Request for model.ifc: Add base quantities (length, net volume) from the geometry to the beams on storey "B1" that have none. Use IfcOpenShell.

First a look at what the model holds.

```python
import ifcopenshell
import ifcopenshell.util.element
import ifcopenshell.util.unit

model = ifcopenshell.open("model.ifc")
print(model.schema)
for unit_type in ("LENGTHUNIT", "AREAUNIT", "VOLUMEUNIT"):
    print(unit_type, ifcopenshell.util.unit.calculate_unit_scale(model, unit_type))
storey = next(s for s in model.by_type("IfcBuildingStorey") if s.Name == "B1")
beams = [e for e in ifcopenshell.util.element.get_decomposition(storey) if e.is_a("IfcBeam")]
for e in sorted(beams, key=lambda e: e.id()):
    print(e.id(), e.is_a(), e.Name, list(ifcopenshell.util.element.get_psets(e, qtos_only=True)), sep=" | ")
```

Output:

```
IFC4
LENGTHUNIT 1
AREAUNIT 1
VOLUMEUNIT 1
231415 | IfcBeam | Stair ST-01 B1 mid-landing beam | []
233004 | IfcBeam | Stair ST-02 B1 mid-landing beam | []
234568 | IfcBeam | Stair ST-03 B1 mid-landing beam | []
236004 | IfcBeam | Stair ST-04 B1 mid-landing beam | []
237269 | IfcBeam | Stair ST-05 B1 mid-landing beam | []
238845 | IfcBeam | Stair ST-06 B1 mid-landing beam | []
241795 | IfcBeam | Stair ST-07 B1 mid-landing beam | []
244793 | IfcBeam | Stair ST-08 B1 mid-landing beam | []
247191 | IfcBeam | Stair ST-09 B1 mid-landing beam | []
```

```python
import ifcopenshell
import ifcopenshell.api.pset
import ifcopenshell.geom
import ifcopenshell.util.element
import ifcopenshell.util.shape
import ifcopenshell.util.unit

model = ifcopenshell.open("model.ifc")
unit_scale = ifcopenshell.util.unit.calculate_unit_scale(model)
volume_scale = ifcopenshell.util.unit.calculate_unit_scale(model, "VOLUMEUNIT")
settings = ifcopenshell.geom.settings()

storey = next(s for s in model.by_type("IfcBuildingStorey") if s.Name == "B1")
beams = [e for e in ifcopenshell.util.element.get_decomposition(storey) if e.is_a("IfcBeam")]

for e in sorted(beams, key=lambda e: e.id()):
    if ifcopenshell.util.element.get_psets(e, qtos_only=True, should_inherit=False):
        continue
    # Geometry comes back in metres, in the element's own axes.
    shape = ifcopenshell.geom.create_shape(settings, e)
    values = {
        "Length": ifcopenshell.util.shape.get_max_xyz(shape.geometry) / unit_scale,
        "NetVolume": ifcopenshell.util.shape.get_volume(shape.geometry) / volume_scale,
    }
    qto = ifcopenshell.api.pset.add_qto(model, product=e, name="Qto_BeamBaseQuantities")
    ifcopenshell.api.pset.edit_qto(model, qto=qto, properties=values)
    print(e.id(), {k: round(v, 3) for k, v in values.items()})

model.write("model_v2.ifc")
```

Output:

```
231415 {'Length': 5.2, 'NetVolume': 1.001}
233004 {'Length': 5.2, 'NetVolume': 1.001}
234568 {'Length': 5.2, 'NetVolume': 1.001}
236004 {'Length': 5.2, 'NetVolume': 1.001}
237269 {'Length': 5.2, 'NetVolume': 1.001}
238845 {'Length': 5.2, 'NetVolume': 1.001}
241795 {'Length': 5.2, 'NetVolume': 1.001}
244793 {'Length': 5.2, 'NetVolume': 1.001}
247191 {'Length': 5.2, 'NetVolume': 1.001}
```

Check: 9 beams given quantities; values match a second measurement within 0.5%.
